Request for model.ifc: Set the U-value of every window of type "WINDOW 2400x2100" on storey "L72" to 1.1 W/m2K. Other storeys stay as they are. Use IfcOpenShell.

First a look at what the model holds.

```python
import ifcopenshell
import ifcopenshell.util.element

model = ifcopenshell.open("model.ifc")
print(model.schema)
storey = next(s for s in model.by_type("IfcBuildingStorey") if s.Name == "L72")
windows = [e for e in ifcopenshell.util.element.get_decomposition(storey) if e.is_a("IfcWindow")]
seen = {}
for e in windows:
    element_type = ifcopenshell.util.element.get_type(e)
    key = (element_type.Name if element_type != e and element_type else None, ifcopenshell.util.element.get_pset(e, "Pset_WindowCommon", "ThermalTransmittance"))
    seen[key] = seen.get(key, 0) + 1
for (name, value), count in sorted(seen.items(), key=str):
    print(count, "x", name, "|", value)
```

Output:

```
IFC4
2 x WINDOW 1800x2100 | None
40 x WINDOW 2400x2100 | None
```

```python
import ifcopenshell
import ifcopenshell.api.pset
import ifcopenshell.util.element

model = ifcopenshell.open("model.ifc")

storey = next(s for s in model.by_type("IfcBuildingStorey") if s.Name == "L72")
windows = [e for e in ifcopenshell.util.element.get_decomposition(storey) if e.is_a("IfcWindow")]

count = 0
for e in windows:
    element_type = ifcopenshell.util.element.get_type(e)
    if element_type in (None, e) or element_type.Name != "WINDOW 2400x2100":
        continue
    found = ifcopenshell.util.element.get_pset(e, "Pset_WindowCommon", should_inherit=False)
    if found:
        pset = model.by_id(found["id"])
        if len(ifcopenshell.util.element.get_elements_by_pset(pset)) > 1:
            pset = ifcopenshell.api.pset.unshare_pset(model, products=[e], pset=pset)[0]
    else:
        pset = ifcopenshell.api.pset.add_pset(model, product=e, name="Pset_WindowCommon")
    ifcopenshell.api.pset.edit_pset(model, pset=pset, properties={"ThermalTransmittance": 1.1})
    count += 1

print(count, "windows updated")

model.write("model_rev.ifc")
```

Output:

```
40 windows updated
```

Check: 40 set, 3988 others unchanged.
